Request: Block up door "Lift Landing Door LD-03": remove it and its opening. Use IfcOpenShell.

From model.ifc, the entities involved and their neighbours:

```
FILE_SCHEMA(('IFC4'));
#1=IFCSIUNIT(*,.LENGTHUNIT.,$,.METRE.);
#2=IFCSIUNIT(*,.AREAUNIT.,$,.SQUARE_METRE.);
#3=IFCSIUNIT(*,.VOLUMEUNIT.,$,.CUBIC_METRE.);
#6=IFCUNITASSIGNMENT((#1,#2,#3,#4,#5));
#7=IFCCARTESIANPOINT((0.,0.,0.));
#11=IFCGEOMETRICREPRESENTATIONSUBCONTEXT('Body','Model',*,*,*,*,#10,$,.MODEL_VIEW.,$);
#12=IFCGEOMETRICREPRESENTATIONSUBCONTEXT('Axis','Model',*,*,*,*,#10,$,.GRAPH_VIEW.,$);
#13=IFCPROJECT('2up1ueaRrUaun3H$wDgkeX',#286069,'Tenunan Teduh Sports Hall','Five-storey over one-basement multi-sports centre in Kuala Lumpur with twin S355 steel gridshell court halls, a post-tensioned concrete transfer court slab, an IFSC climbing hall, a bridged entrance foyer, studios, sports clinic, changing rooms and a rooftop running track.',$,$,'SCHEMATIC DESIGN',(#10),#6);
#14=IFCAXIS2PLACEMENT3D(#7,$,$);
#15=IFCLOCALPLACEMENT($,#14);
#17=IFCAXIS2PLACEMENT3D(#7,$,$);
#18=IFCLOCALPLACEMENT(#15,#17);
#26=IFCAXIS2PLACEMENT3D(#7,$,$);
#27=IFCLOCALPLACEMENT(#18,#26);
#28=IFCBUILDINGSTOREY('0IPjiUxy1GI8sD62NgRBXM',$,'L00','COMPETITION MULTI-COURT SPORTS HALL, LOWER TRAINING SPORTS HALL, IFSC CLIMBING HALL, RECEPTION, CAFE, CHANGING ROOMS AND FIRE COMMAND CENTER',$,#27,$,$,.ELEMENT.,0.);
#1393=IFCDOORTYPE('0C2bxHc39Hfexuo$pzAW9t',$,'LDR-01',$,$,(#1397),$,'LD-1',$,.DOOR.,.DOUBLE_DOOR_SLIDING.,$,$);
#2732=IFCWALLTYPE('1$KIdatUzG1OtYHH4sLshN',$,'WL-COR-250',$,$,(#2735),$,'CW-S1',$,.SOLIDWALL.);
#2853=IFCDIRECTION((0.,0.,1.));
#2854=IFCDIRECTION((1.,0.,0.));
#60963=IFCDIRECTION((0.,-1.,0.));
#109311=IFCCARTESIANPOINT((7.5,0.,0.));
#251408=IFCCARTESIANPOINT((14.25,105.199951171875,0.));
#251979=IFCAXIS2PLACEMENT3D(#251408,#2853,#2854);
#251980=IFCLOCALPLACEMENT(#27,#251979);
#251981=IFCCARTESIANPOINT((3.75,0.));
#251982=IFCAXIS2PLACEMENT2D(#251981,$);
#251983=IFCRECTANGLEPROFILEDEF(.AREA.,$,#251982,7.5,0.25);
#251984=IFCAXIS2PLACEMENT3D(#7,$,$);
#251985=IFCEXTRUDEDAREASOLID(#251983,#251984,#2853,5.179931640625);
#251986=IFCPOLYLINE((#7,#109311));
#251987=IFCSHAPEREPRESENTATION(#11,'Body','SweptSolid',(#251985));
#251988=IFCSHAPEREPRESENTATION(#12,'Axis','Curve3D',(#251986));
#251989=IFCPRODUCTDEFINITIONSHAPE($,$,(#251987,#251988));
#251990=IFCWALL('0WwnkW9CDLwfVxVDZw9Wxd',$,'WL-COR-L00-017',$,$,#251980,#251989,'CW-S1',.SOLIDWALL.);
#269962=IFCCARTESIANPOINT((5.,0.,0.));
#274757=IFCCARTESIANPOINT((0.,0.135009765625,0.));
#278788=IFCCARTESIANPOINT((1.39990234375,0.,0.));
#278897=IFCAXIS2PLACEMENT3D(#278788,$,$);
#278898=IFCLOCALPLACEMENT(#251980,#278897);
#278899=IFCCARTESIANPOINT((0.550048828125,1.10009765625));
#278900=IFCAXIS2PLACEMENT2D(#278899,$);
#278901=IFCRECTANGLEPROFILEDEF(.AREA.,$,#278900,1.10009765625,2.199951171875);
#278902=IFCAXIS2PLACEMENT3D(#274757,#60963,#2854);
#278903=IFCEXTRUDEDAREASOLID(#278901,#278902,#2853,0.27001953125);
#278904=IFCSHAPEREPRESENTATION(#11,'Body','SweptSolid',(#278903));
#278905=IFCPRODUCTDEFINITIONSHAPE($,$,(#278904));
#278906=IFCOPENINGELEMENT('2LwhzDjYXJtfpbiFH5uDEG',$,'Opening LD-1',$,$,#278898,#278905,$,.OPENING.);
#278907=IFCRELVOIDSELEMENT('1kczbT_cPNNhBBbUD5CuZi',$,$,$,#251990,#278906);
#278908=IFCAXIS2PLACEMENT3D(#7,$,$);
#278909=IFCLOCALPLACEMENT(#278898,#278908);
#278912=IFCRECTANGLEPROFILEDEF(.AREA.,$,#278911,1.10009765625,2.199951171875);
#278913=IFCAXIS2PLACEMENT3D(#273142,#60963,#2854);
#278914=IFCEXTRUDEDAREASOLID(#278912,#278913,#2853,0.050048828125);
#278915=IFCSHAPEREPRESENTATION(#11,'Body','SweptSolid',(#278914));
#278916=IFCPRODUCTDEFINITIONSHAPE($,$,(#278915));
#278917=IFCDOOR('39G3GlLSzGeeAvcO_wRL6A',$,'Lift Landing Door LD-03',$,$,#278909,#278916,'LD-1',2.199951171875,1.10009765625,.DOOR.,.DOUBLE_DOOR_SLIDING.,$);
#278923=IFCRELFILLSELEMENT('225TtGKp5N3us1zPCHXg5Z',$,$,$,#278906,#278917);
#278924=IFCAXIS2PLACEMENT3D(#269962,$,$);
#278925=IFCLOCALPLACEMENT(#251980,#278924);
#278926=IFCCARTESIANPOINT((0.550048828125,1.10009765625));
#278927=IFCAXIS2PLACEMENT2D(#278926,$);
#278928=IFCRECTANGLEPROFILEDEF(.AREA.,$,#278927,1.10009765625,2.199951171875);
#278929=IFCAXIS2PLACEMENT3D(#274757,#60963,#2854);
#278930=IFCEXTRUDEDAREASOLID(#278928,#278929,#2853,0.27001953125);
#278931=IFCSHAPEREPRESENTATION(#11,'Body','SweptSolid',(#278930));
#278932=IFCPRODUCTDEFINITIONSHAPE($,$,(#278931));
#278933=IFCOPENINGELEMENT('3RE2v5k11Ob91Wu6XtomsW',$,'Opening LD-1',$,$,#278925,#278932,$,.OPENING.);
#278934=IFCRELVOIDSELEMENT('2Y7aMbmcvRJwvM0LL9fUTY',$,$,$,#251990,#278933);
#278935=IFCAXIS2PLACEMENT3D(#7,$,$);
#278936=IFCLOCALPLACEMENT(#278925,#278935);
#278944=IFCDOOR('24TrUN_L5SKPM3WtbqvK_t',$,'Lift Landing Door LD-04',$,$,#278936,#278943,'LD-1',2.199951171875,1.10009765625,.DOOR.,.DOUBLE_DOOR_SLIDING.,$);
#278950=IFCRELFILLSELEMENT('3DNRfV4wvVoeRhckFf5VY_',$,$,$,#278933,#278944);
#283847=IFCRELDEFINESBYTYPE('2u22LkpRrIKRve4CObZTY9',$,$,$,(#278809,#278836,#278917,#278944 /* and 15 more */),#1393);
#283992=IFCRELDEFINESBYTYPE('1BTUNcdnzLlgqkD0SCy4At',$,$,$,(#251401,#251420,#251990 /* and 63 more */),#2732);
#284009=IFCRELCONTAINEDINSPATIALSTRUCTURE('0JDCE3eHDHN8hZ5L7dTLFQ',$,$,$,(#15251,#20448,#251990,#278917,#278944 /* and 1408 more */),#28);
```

```python
import ifcopenshell
import ifcopenshell.api.feature
import ifcopenshell.api.root
import ifcopenshell.geom
import ifcopenshell.util.shape

model = ifcopenshell.open("model.ifc")
settings = ifcopenshell.geom.settings()


def volume(element):
    """Net volume in cubic metres, openings subtracted."""
    shape = ifcopenshell.geom.create_shape(settings, element)
    return ifcopenshell.util.shape.get_volume(shape.geometry)


door = model.by_guid("39G3GlLSzGeeAvcO_wRL6A")
opening = door.FillsVoids[0].RelatingOpeningElement
wall = opening.VoidsElements[0].RelatingBuildingElement
before = volume(wall)

ifcopenshell.api.root.remove_product(model, product=door)
ifcopenshell.api.feature.remove_feature(model, feature=opening)

after = volume(wall)

print(f"wall volume {before:.3f} -> {after:.3f} m3")

model.write("model_rev.ifc")
```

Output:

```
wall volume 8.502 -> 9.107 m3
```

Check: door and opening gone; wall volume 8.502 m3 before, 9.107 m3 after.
